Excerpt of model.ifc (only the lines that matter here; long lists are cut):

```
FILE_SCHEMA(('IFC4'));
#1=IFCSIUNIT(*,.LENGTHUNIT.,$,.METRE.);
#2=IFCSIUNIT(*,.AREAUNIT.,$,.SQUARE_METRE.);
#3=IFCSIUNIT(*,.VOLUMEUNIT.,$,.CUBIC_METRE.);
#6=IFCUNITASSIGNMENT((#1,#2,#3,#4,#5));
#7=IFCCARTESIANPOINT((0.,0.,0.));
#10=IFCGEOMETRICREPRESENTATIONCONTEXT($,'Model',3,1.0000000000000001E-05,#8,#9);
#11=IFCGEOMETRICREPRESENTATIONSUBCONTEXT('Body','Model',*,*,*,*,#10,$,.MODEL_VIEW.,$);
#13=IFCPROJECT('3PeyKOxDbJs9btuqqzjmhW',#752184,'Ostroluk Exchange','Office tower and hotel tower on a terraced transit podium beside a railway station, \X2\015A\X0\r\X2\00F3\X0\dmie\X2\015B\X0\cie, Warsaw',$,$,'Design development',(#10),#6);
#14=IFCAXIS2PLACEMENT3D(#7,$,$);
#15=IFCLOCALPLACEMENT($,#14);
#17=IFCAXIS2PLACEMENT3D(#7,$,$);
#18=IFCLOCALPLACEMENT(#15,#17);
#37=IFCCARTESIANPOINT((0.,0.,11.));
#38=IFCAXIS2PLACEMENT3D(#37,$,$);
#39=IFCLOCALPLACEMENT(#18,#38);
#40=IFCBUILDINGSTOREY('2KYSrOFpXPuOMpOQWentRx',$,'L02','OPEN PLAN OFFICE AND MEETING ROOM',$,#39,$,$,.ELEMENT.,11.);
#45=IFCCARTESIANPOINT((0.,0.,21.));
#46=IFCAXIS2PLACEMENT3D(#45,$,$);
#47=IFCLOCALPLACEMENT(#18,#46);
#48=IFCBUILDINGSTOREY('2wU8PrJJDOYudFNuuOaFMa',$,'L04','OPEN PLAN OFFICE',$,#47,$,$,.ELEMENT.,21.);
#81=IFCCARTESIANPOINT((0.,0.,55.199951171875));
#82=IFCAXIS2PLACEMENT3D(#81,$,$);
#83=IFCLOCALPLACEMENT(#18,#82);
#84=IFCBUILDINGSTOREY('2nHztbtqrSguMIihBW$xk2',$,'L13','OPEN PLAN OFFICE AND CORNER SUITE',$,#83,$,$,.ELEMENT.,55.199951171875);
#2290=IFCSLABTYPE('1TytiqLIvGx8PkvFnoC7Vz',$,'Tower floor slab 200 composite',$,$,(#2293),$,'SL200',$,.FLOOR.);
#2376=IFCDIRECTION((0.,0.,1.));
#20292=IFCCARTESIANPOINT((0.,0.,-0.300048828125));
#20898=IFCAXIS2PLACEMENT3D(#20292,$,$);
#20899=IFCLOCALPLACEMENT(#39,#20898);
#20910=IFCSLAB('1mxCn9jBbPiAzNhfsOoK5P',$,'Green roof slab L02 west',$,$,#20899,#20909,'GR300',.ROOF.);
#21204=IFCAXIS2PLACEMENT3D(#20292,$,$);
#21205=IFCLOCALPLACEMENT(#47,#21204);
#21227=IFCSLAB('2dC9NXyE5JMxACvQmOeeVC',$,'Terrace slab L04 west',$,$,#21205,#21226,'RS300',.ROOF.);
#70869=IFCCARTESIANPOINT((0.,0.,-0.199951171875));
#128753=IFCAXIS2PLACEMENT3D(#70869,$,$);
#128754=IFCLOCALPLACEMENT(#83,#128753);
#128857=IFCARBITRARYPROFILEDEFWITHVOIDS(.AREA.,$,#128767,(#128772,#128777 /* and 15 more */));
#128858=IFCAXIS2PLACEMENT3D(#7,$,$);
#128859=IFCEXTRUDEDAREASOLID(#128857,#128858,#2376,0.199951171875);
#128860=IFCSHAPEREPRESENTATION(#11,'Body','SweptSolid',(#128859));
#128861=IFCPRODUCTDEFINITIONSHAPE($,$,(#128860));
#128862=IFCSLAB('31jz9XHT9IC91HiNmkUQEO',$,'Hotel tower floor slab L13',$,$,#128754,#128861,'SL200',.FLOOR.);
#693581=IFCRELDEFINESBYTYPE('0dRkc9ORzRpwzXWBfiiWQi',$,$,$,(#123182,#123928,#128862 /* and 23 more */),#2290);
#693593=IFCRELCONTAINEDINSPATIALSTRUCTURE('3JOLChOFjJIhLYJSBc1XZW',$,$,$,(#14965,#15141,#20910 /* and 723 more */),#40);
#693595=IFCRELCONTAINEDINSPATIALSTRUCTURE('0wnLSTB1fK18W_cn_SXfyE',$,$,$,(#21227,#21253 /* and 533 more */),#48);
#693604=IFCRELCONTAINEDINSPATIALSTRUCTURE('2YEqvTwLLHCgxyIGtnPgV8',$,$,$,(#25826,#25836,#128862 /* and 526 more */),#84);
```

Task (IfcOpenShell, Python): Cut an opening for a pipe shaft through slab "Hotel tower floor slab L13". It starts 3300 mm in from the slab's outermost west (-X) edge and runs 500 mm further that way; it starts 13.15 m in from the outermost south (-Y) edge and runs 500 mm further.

```python
import numpy as np
import ifcopenshell
import ifcopenshell.api.feature
import ifcopenshell.api.geometry
import ifcopenshell.api.root
import ifcopenshell.geom
import ifcopenshell.util.placement
import ifcopenshell.util.representation
import ifcopenshell.util.shape
import ifcopenshell.util.unit

model = ifcopenshell.open("model.ifc")
unit_scale = ifcopenshell.util.unit.calculate_unit_scale(model)
settings = ifcopenshell.geom.settings()


def volume(element):
    """Net volume in cubic metres, openings subtracted."""
    shape = ifcopenshell.geom.create_shape(settings, element)
    return ifcopenshell.util.shape.get_volume(shape.geometry)


slab = model.by_id(128862)
before = volume(slab)

# Extent in the slab's own axes, in metres. The edges named are its -X and -Y sides.
slab_shape = ifcopenshell.geom.create_shape(settings, slab)
vertices = ifcopenshell.util.shape.get_vertices(slab_shape.geometry)
x_min, y_min, bottom = vertices.min(axis=0)
top = vertices[:, 2].max()

opening = ifcopenshell.api.root.create_entity(model, ifc_class="IfcOpeningElement", name="Pipe shaft opening", predefined_type="OPENING")
context = ifcopenshell.util.representation.get_context(model, "Model", "Body", "MODEL_VIEW")
width, depth = 0.5, 0.5
outline = [(0.0, 0.0), (width, 0.0), (width, depth), (0.0, depth), (0.0, 0.0)]
# Overshoot both faces by 50 mm so the cut is clean.
shape = ifcopenshell.api.geometry.add_slab_representation(
    model, context=context, depth=top - bottom + 0.1, polyline=outline
)
ifcopenshell.api.geometry.assign_representation(model, product=opening, representation=shape)

matrix = ifcopenshell.util.placement.get_local_placement(slab.ObjectPlacement)
matrix[:, 3] = matrix @ np.append(np.array([x_min + 3.3, y_min + 13.15, bottom - 0.05]) / unit_scale, 1.0)
ifcopenshell.api.geometry.edit_object_placement(model, product=opening, matrix=matrix, is_si=False)
ifcopenshell.api.feature.add_feature(model, feature=opening, element=slab)

after = volume(slab)

print(f"slab volume {before:.3f} -> {after:.3f} m3")

model.write("model_v2.ifc")
```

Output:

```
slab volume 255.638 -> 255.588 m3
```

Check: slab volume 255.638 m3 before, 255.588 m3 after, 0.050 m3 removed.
